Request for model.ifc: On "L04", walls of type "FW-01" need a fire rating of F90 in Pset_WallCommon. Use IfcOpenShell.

First a look at what the model holds.

```python
import ifcopenshell
import ifcopenshell.util.element

model = ifcopenshell.open("model.ifc")
print(model.schema)
storey = next(s for s in model.by_type("IfcBuildingStorey") if s.Name == "L04")
walls = [e for e in ifcopenshell.util.element.get_decomposition(storey) if e.is_a("IfcWall")]
seen = {}
for e in walls:
    element_type = ifcopenshell.util.element.get_type(e)
    key = (element_type.Name if element_type != e and element_type else None, ifcopenshell.util.element.get_pset(e, "Pset_WallCommon", "FireRating"))
    seen[key] = seen.get(key, 0) + 1
for (name, value), count in sorted(seen.items(), key=str):
    print(count, "x", name, "|", value)
```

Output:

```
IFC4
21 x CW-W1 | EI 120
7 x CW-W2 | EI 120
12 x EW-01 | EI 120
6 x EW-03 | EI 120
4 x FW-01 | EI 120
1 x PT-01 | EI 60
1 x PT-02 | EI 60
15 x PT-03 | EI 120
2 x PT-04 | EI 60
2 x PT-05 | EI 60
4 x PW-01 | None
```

```python
import ifcopenshell
import ifcopenshell.api.pset
import ifcopenshell.util.element

model = ifcopenshell.open("model.ifc")

storey = next(s for s in model.by_type("IfcBuildingStorey") if s.Name == "L04")
walls = [e for e in ifcopenshell.util.element.get_decomposition(storey) if e.is_a("IfcWall")]

count = 0
for e in walls:
    element_type = ifcopenshell.util.element.get_type(e)
    if element_type in (None, e) or element_type.Name != "FW-01":
        continue
    # add_pset returns the element's existing set when there is one.
    pset = ifcopenshell.api.pset.add_pset(model, product=e, name="Pset_WallCommon")
    ifcopenshell.api.pset.edit_pset(model, pset=pset, properties={"FireRating": "F90"})
    count += 1

print(count, "walls updated")

model.write("model-out.ifc")
```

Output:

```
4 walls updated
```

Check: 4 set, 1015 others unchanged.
